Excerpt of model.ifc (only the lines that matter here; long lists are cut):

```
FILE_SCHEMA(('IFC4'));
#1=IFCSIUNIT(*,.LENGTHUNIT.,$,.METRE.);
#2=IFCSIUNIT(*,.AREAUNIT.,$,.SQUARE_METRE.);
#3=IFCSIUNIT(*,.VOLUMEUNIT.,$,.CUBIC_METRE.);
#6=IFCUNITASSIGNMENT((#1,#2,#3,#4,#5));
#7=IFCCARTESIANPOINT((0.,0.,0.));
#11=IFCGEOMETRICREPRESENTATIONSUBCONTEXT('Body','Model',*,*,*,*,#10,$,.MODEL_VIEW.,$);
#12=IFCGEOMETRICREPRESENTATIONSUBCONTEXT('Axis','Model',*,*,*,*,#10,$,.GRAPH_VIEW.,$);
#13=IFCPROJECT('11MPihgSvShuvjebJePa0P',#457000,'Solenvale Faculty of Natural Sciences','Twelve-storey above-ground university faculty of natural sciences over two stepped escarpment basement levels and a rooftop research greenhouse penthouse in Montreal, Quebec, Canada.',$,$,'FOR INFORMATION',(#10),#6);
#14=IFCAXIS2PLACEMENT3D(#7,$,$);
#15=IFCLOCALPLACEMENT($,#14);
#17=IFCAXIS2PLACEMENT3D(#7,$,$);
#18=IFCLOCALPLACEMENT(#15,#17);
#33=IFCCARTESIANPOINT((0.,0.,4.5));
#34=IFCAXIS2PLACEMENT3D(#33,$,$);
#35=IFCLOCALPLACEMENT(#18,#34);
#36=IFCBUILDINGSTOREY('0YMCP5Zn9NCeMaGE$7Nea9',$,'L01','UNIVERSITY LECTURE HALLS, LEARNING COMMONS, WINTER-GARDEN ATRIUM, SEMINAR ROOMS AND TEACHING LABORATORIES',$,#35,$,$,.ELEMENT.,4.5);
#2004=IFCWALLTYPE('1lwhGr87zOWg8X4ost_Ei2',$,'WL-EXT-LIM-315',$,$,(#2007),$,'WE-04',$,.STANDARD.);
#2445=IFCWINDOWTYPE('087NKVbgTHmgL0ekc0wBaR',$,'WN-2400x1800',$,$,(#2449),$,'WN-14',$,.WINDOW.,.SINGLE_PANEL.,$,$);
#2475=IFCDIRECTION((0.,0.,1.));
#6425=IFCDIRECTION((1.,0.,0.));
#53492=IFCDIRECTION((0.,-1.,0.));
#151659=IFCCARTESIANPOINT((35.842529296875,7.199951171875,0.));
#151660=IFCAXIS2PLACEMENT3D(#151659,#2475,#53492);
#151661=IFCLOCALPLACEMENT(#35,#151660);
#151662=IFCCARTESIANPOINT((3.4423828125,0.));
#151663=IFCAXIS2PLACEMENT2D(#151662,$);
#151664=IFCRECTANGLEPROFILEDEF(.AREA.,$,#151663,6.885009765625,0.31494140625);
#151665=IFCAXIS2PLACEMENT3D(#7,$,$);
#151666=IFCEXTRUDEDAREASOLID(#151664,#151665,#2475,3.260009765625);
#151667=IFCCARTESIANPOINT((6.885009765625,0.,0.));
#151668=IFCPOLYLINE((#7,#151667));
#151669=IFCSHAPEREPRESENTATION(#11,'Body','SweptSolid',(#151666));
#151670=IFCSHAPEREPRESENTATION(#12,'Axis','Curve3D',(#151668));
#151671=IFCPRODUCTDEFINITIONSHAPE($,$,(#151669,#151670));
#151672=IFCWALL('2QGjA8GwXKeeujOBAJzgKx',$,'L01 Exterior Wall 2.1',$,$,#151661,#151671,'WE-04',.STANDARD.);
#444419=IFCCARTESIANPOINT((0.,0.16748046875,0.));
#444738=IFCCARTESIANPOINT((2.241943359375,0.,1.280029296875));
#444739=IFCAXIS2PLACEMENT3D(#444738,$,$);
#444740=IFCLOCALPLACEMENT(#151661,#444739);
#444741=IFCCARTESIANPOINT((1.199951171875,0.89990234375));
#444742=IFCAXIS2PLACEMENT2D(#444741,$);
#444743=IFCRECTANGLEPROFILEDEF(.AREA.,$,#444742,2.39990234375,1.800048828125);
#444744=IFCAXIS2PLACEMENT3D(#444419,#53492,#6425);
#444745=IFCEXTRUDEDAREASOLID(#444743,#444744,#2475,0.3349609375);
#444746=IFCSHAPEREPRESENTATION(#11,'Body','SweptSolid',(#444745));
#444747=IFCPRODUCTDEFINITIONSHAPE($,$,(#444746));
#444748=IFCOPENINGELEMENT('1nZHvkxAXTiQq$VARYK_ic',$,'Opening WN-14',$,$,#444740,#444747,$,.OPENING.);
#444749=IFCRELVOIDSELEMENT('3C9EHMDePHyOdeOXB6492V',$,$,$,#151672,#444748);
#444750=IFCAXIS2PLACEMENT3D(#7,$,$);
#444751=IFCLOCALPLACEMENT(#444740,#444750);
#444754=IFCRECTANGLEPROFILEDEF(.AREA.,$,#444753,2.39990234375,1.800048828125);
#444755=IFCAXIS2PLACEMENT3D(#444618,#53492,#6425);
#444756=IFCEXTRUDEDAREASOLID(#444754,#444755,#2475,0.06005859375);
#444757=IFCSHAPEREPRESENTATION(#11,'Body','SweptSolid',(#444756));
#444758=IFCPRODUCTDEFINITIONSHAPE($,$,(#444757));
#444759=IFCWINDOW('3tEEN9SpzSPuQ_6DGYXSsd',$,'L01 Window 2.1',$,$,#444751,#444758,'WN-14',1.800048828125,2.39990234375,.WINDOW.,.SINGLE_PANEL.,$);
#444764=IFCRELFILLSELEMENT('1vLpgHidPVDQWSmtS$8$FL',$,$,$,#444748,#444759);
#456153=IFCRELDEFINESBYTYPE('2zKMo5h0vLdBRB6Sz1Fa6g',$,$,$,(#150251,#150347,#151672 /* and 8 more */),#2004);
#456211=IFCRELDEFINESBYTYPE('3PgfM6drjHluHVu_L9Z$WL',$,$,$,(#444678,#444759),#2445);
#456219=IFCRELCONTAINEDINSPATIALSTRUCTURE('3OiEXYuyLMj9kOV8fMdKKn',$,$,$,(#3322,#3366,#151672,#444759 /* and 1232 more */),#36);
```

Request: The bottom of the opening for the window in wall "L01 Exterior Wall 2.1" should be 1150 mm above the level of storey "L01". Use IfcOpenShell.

```python
import numpy as np
import ifcopenshell
import ifcopenshell.api.geometry
import ifcopenshell.geom
import ifcopenshell.util.element
import ifcopenshell.util.placement
import ifcopenshell.util.shape
import ifcopenshell.util.unit

model = ifcopenshell.open("model.ifc")
unit_scale = ifcopenshell.util.unit.calculate_unit_scale(model)

window = model.by_id(444759)
opening = window.FillsVoids[0].RelatingOpeningElement
storey = ifcopenshell.util.element.get_container(window, ifc_class="IfcBuildingStorey")
level = ifcopenshell.util.placement.get_local_placement(storey.ObjectPlacement)[2, 3]

# The opening's origin need not be at the sill, so measure its lowest point.
shape = ifcopenshell.geom.create_shape(ifcopenshell.geom.settings(), opening)
bottom = ifcopenshell.util.shape.get_shape_bottom_elevation(shape, shape.geometry) / unit_scale
dz = level + 1.15 - bottom

shift = np.array([0.0, 0.0, dz])
# The window is placed relative to its opening, so it follows when the opening moves.
matrix = ifcopenshell.util.placement.get_local_placement(opening.ObjectPlacement)
matrix[:3, 3] += shift
ifcopenshell.api.geometry.edit_object_placement(
    model, product=opening, matrix=matrix, is_si=False, should_transform_children=True
)

print(f"moved by {dz * unit_scale:+.3f} m")

model.write("model_edited.ifc")
```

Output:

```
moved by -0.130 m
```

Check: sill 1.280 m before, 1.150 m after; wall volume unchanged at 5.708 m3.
